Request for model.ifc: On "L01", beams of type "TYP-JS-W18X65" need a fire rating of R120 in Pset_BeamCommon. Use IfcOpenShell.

First a look at what the model holds.

```python
import ifcopenshell
import ifcopenshell.util.element

model = ifcopenshell.open("model.ifc")
print(model.schema)
storey = next(s for s in model.by_type("IfcBuildingStorey") if s.Name == "L01")
beams = [e for e in ifcopenshell.util.element.get_decomposition(storey) if e.is_a("IfcBeam")]
seen = {}
for e in beams:
    element_type = ifcopenshell.util.element.get_type(e)
    key = (element_type.Name if element_type != e and element_type else None, ifcopenshell.util.element.get_pset(e, "Pset_BeamCommon", "FireRating"))
    seen[key] = seen.get(key, 0) + 1
for (name, value), count in sorted(seen.items(), key=str):
    print(count, "x", name, "|", value)
```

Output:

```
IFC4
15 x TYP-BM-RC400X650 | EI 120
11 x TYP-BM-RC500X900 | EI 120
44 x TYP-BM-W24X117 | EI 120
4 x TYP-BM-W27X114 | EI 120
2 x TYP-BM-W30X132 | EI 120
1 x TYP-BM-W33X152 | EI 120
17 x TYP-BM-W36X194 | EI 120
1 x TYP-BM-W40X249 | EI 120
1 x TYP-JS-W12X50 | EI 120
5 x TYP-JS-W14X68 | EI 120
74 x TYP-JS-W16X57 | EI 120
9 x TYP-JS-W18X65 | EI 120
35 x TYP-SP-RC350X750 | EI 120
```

```python
import ifcopenshell
import ifcopenshell.api.pset
import ifcopenshell.util.element

model = ifcopenshell.open("model.ifc")

storey = next(s for s in model.by_type("IfcBuildingStorey") if s.Name == "L01")
beams = [e for e in ifcopenshell.util.element.get_decomposition(storey) if e.is_a("IfcBeam")]

count = 0
for e in beams:
    element_type = ifcopenshell.util.element.get_type(e)
    if element_type in (None, e) or element_type.Name != "TYP-JS-W18X65":
        continue
    # add_pset returns the element's existing set when there is one.
    pset = ifcopenshell.api.pset.add_pset(model, product=e, name="Pset_BeamCommon")
    ifcopenshell.api.pset.edit_pset(model, pset=pset, properties={"FireRating": "R120"})
    count += 1

print(count, "beams updated")

model.write("model_rev.ifc")
```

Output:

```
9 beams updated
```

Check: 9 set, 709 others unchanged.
